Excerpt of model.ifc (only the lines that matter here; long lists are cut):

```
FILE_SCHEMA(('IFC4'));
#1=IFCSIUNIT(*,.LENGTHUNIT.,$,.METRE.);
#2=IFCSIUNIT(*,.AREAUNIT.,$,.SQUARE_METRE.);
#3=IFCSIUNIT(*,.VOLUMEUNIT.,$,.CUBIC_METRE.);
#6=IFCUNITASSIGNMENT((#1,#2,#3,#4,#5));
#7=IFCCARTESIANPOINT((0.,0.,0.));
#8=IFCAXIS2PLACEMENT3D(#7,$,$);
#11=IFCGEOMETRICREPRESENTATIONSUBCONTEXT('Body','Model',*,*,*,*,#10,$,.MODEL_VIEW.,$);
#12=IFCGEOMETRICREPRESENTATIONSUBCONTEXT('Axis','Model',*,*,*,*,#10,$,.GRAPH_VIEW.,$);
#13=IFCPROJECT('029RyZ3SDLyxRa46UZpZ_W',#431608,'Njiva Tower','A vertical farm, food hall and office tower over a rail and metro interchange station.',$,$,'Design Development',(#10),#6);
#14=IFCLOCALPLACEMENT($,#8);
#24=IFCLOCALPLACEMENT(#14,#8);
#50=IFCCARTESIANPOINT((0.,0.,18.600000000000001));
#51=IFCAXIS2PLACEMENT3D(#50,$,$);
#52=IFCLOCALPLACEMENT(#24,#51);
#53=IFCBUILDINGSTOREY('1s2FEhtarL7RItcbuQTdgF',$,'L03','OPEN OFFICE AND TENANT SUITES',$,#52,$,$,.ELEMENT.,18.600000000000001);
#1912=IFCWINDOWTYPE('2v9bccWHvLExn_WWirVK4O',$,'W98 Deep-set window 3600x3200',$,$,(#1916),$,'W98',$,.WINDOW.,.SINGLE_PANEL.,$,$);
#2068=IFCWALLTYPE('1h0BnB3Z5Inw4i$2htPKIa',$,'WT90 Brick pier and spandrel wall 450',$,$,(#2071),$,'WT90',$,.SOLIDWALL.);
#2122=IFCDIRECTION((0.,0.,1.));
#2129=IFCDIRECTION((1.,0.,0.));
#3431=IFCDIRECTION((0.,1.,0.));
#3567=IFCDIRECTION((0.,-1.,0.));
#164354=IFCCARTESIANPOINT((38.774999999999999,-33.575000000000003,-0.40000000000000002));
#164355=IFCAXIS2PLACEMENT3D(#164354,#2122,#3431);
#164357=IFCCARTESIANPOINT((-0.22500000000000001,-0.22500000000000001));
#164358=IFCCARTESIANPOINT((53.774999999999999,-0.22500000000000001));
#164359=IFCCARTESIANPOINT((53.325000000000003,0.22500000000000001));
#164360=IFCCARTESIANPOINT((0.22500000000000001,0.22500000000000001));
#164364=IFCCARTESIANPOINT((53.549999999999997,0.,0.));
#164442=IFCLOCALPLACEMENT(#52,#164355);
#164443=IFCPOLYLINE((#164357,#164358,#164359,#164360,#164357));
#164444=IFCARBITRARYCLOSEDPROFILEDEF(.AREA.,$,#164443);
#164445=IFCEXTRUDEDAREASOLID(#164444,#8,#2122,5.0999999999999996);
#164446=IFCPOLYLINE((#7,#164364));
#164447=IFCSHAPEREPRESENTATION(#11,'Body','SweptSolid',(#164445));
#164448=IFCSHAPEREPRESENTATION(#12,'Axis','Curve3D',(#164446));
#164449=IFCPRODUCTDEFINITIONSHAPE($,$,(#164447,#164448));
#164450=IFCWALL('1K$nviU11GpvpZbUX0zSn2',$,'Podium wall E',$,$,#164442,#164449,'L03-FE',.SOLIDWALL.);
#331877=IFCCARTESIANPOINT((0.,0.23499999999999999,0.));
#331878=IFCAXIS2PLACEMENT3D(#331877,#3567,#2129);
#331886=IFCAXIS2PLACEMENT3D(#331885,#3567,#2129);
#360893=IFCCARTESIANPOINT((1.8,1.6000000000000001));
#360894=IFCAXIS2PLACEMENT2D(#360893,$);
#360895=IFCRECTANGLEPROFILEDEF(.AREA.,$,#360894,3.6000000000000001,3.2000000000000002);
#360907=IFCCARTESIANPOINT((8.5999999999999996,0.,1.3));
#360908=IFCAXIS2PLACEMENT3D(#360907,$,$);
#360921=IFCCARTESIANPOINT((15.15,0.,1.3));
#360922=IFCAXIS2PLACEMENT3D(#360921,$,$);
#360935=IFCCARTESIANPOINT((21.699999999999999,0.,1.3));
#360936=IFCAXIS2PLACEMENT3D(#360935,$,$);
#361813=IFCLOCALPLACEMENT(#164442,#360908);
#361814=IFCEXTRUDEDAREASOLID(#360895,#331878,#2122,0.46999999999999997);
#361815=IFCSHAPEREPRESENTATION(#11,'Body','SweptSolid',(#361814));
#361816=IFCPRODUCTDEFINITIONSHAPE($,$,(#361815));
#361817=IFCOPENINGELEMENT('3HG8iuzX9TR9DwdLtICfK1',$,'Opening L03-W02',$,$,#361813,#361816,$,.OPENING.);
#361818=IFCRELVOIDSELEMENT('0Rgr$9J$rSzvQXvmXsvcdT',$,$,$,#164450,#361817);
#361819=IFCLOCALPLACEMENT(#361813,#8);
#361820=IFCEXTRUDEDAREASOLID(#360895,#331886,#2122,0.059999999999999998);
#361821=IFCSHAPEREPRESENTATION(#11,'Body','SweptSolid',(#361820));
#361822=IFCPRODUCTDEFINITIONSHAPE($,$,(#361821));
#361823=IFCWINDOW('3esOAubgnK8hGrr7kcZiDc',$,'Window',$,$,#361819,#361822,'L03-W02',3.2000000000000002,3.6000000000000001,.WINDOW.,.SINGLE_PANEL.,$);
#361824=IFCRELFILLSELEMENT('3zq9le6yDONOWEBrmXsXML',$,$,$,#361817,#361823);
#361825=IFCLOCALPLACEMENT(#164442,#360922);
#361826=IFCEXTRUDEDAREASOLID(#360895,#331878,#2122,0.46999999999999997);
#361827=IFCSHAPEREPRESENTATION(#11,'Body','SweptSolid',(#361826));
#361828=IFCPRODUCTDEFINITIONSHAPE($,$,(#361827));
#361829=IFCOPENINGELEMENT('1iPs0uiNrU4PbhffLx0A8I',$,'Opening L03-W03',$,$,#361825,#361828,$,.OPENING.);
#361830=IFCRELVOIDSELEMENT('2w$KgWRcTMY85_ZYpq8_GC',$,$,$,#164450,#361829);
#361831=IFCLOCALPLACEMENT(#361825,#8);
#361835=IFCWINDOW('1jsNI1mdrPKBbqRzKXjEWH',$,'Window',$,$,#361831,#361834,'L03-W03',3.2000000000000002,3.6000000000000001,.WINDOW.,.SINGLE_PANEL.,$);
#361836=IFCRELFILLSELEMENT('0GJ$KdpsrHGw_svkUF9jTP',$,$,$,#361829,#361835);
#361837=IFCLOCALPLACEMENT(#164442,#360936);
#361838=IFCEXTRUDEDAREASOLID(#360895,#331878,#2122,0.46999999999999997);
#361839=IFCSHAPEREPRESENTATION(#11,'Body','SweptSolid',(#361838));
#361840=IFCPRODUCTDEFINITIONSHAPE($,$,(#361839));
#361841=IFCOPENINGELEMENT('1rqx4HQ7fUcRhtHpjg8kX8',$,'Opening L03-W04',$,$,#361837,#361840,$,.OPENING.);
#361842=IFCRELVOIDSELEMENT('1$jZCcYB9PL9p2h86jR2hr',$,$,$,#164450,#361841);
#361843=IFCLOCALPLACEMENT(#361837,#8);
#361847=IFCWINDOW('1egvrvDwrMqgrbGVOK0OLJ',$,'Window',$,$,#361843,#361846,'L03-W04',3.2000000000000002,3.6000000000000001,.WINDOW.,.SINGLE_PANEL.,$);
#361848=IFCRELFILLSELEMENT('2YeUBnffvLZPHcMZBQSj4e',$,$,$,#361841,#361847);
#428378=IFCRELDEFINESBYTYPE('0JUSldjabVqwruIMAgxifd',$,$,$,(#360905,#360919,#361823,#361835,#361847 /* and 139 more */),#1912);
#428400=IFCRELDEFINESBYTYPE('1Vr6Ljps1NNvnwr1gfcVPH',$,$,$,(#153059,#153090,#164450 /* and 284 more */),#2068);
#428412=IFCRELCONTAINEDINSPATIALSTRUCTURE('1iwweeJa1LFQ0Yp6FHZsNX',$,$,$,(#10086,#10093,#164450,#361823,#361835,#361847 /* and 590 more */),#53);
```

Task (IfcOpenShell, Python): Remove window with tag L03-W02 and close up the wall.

```python
import ifcopenshell
import ifcopenshell.api.feature
import ifcopenshell.api.root
import ifcopenshell.geom
import ifcopenshell.util.shape

model = ifcopenshell.open("model.ifc")
settings = ifcopenshell.geom.settings()


def volume(element):
    """Net volume in cubic metres, openings subtracted."""
    shape = ifcopenshell.geom.create_shape(settings, element)
    return ifcopenshell.util.shape.get_volume(shape.geometry)


window = model.by_guid("3esOAubgnK8hGrr7kcZiDc")
opening = window.FillsVoids[0].RelatingOpeningElement
wall = opening.VoidsElements[0].RelatingBuildingElement
before = volume(wall)

ifcopenshell.api.root.remove_product(model, product=window)
ifcopenshell.api.feature.remove_feature(model, feature=opening)

after = volume(wall)

print(f"wall volume {before:.3f} -> {after:.3f} m3")

model.write("model_edited.ifc")
```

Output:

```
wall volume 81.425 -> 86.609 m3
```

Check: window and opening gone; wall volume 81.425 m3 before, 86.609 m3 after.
